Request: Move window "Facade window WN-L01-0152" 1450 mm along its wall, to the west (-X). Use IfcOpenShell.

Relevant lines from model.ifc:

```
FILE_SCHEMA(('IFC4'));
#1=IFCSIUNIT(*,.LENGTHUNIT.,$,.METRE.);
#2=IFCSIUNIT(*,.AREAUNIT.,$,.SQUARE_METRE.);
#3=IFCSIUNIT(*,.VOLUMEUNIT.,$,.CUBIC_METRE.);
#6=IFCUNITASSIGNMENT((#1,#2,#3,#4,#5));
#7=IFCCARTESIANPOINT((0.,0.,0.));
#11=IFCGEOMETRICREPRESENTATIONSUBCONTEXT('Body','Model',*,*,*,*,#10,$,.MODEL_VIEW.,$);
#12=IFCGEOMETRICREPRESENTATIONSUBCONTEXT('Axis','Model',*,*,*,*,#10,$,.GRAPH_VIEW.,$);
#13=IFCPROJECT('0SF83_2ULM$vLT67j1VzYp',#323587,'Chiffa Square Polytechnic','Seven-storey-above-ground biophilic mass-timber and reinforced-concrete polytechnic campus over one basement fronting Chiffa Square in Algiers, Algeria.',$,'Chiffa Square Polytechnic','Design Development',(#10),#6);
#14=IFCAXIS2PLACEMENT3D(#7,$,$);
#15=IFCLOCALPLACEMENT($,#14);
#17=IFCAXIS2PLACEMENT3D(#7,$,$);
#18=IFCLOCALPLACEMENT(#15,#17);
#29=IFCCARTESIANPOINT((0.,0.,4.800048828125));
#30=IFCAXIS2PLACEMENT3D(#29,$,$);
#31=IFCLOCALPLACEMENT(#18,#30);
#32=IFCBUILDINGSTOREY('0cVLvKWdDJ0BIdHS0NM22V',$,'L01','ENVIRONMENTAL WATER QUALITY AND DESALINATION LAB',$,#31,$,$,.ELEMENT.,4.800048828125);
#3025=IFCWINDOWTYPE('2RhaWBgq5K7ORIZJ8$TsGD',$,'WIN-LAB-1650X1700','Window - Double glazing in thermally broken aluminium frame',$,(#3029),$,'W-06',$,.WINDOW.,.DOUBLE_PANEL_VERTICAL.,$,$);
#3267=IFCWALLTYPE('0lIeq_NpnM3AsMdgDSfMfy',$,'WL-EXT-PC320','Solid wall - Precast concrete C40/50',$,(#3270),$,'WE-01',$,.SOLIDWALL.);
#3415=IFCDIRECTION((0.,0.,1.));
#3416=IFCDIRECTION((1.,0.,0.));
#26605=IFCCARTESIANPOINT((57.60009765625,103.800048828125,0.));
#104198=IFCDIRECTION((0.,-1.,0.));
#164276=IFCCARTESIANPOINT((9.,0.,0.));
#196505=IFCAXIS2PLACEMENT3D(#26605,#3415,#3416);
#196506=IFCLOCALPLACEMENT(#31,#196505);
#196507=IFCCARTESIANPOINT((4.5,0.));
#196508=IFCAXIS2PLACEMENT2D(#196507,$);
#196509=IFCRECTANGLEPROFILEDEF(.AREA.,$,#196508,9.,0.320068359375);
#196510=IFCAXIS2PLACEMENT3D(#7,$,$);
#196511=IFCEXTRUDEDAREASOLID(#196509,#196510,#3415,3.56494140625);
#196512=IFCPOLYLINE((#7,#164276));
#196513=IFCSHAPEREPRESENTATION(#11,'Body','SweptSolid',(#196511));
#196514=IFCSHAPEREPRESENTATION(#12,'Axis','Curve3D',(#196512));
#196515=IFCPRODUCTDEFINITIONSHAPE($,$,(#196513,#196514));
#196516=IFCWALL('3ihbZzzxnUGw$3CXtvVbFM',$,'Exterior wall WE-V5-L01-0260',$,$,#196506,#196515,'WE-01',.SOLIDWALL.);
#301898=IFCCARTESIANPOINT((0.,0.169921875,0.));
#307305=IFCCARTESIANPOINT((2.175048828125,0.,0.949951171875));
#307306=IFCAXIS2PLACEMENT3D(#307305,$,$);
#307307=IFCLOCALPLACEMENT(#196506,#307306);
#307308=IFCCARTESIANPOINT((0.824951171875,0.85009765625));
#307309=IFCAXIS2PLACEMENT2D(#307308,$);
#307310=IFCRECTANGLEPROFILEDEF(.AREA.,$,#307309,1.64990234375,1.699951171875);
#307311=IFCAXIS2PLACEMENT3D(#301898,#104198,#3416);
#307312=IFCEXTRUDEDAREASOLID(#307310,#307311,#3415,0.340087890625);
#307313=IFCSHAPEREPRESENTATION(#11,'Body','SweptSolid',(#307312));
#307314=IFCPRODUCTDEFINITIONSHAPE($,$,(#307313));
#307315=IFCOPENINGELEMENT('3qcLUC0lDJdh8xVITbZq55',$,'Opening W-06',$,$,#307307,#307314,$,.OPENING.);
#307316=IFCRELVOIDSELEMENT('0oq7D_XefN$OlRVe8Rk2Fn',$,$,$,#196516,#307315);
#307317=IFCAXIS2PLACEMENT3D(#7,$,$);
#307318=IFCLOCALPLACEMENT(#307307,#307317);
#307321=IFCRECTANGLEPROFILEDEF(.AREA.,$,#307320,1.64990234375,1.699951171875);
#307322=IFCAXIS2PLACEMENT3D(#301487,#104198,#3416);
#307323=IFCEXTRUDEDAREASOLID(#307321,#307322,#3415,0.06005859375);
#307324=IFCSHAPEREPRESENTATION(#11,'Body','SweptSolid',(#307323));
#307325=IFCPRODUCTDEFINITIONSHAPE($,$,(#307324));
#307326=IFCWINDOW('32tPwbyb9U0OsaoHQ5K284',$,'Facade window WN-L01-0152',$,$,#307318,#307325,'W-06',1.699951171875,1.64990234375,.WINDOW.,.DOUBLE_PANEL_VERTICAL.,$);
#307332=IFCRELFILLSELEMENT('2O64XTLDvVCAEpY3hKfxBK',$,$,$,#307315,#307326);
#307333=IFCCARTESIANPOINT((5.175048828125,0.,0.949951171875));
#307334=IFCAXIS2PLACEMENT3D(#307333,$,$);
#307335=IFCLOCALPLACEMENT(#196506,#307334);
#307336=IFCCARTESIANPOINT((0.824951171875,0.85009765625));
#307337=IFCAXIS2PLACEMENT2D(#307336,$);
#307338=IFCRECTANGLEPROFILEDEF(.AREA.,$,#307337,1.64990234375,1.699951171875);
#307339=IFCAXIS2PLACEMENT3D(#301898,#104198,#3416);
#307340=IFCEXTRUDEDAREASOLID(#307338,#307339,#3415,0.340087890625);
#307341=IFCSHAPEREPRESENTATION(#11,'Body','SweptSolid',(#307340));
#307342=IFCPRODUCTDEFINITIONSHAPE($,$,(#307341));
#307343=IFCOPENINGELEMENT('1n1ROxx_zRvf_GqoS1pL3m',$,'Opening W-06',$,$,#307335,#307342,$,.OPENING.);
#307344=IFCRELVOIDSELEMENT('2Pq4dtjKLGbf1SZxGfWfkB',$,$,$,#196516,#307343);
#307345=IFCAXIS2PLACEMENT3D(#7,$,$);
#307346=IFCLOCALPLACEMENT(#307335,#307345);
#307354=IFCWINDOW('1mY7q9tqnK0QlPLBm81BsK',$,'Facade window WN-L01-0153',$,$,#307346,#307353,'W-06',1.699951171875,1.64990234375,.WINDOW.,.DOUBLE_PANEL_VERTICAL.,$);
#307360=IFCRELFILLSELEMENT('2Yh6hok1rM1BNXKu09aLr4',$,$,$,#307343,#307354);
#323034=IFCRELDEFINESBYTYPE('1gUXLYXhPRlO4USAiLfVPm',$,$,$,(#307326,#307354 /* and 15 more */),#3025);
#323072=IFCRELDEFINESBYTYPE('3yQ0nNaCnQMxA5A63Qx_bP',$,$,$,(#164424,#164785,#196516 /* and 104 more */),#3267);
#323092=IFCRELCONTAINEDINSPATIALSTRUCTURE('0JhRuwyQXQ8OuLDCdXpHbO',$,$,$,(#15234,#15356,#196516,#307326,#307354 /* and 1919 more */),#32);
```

```python
import ifcopenshell
import ifcopenshell.api.geometry
import ifcopenshell.util.placement
import ifcopenshell.util.unit

model = ifcopenshell.open("model.ifc")
unit_scale = ifcopenshell.util.unit.calculate_unit_scale(model)

window = model.by_guid("32tPwbyb9U0OsaoHQ5K284")
opening = window.FillsVoids[0].RelatingOpeningElement
wall = opening.VoidsElements[0].RelatingBuildingElement

wall_matrix = ifcopenshell.util.placement.get_local_placement(wall.ObjectPlacement)
shift = wall_matrix[:3, 0] * -1.45 / unit_scale
before = ifcopenshell.util.placement.get_local_placement(window.ObjectPlacement)[:3, 3].copy()

# The window is placed relative to its opening, so it follows when the opening moves.
matrix = ifcopenshell.util.placement.get_local_placement(opening.ObjectPlacement)
matrix[:3, 3] += shift
ifcopenshell.api.geometry.edit_object_placement(
    model, product=opening, matrix=matrix, is_si=False, should_transform_children=True
)

after = ifcopenshell.util.placement.get_local_placement(window.ObjectPlacement)[:3, 3]
print("window moved by", (after - before).round(3) + 0.0)

model.write("model_v2.ifc")
```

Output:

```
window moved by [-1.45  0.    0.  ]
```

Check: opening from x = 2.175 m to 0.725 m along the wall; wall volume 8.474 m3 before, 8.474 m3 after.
